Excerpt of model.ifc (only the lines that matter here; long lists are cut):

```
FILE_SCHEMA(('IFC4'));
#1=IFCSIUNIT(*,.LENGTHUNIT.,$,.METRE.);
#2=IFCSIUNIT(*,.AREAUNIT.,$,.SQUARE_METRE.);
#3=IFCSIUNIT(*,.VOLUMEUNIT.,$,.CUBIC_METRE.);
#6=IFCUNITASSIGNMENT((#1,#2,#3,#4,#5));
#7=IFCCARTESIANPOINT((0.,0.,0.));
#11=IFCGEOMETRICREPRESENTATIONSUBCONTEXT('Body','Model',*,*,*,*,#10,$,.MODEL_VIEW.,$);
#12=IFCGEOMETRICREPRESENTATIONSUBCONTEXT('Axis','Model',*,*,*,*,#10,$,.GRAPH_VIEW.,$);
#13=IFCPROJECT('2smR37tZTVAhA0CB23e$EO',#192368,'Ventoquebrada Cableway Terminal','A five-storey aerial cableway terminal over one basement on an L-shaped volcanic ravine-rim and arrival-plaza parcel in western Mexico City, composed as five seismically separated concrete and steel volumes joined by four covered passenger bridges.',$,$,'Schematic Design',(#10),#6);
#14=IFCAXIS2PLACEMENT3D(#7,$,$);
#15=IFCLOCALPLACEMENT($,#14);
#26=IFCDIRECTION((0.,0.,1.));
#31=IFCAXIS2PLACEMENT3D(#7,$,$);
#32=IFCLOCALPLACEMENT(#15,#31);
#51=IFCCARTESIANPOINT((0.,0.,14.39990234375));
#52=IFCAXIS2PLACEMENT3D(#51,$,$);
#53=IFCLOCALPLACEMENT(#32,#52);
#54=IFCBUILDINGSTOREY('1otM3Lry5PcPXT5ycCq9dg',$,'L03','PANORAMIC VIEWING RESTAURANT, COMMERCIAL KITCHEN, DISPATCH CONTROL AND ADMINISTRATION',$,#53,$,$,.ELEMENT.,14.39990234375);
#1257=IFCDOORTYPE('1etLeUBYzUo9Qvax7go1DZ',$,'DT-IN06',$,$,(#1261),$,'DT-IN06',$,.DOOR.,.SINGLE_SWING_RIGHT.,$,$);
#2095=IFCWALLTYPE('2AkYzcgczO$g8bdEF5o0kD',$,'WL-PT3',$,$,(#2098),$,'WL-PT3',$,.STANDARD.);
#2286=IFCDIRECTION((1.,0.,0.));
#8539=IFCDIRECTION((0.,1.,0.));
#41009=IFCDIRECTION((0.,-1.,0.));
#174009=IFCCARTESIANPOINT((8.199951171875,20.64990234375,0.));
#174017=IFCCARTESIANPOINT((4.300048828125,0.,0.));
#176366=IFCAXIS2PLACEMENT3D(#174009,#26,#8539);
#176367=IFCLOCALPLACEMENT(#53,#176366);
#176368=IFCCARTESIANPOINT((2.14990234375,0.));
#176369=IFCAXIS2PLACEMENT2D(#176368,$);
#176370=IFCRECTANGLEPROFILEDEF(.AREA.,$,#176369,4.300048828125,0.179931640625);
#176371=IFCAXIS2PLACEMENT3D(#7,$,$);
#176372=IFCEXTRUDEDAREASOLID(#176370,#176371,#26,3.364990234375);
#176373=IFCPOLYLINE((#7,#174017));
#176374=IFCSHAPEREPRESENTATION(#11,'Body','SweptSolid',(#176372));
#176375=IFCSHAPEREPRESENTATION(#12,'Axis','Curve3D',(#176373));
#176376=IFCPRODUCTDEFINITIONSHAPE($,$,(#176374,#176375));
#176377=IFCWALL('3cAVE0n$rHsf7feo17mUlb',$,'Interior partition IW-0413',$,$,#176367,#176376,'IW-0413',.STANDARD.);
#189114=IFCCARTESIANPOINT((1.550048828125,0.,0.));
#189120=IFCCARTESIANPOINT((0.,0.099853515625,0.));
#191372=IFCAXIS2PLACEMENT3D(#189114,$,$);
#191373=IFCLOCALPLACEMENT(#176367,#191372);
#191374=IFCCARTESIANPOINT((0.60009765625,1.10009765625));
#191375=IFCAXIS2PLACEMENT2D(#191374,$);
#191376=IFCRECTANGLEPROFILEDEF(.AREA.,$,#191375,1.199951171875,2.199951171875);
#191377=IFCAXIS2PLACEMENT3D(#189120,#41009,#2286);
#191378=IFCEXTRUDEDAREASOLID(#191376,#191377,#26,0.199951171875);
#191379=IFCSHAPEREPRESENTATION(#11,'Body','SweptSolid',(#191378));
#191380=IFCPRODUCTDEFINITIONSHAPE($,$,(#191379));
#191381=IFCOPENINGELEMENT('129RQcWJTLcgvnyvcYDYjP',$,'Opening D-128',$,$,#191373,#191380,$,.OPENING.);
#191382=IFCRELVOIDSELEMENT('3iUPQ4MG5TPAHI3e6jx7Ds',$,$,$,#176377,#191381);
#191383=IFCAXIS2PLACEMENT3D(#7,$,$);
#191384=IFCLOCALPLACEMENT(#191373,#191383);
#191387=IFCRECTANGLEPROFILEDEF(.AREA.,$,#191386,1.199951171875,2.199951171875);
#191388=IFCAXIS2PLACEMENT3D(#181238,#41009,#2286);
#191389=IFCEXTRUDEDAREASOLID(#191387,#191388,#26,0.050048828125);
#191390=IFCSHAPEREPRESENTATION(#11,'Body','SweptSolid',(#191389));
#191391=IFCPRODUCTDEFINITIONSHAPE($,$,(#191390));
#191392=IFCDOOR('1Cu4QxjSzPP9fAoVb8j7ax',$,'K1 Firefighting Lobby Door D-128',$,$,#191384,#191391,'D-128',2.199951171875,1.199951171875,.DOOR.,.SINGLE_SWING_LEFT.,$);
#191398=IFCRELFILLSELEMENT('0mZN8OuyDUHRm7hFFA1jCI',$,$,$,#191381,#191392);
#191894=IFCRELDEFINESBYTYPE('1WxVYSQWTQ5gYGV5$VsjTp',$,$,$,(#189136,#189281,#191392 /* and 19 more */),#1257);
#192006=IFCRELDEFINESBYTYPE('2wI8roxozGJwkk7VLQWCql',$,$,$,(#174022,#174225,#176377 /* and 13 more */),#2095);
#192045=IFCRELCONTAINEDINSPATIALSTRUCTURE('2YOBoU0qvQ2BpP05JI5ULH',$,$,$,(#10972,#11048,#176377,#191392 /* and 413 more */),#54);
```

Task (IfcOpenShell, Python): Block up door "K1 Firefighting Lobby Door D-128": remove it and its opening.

```python
import ifcopenshell
import ifcopenshell.api.feature
import ifcopenshell.api.root
import ifcopenshell.geom
import ifcopenshell.util.shape

model = ifcopenshell.open("model.ifc")
settings = ifcopenshell.geom.settings()


def volume(element):
    """Net volume in cubic metres, openings subtracted."""
    shape = ifcopenshell.geom.create_shape(settings, element)
    return ifcopenshell.util.shape.get_volume(shape.geometry)


door = model.by_guid("1Cu4QxjSzPP9fAoVb8j7ax")
opening = door.FillsVoids[0].RelatingOpeningElement
wall = opening.VoidsElements[0].RelatingBuildingElement
before = volume(wall)

ifcopenshell.api.root.remove_product(model, product=door)
ifcopenshell.api.feature.remove_feature(model, feature=opening)

after = volume(wall)

print(f"wall volume {before:.3f} -> {after:.3f} m3")

model.write("model-out.ifc")
```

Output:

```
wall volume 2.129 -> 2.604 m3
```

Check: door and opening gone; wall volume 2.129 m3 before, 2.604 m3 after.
